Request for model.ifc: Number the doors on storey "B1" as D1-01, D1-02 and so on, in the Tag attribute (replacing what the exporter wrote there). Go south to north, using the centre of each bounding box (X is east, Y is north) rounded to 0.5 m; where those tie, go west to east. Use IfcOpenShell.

First a look at what the model holds.

```python
import ifcopenshell
import ifcopenshell.util.element
import ifcopenshell.util.placement

model = ifcopenshell.open("model.ifc")
print(model.schema)
storey = next(s for s in model.by_type("IfcBuildingStorey") if s.Name == "B1")
doors = [e for e in ifcopenshell.util.element.get_decomposition(storey) if e.is_a("IfcDoor")]
for e in sorted(doors, key=lambda e: e.id()):
    origin = ifcopenshell.util.placement.get_local_placement(e.ObjectPlacement)[:3, 3]
    print(e.id(), e.Tag, e.Name, origin.round(2) + 0.0, sep=" | ")
```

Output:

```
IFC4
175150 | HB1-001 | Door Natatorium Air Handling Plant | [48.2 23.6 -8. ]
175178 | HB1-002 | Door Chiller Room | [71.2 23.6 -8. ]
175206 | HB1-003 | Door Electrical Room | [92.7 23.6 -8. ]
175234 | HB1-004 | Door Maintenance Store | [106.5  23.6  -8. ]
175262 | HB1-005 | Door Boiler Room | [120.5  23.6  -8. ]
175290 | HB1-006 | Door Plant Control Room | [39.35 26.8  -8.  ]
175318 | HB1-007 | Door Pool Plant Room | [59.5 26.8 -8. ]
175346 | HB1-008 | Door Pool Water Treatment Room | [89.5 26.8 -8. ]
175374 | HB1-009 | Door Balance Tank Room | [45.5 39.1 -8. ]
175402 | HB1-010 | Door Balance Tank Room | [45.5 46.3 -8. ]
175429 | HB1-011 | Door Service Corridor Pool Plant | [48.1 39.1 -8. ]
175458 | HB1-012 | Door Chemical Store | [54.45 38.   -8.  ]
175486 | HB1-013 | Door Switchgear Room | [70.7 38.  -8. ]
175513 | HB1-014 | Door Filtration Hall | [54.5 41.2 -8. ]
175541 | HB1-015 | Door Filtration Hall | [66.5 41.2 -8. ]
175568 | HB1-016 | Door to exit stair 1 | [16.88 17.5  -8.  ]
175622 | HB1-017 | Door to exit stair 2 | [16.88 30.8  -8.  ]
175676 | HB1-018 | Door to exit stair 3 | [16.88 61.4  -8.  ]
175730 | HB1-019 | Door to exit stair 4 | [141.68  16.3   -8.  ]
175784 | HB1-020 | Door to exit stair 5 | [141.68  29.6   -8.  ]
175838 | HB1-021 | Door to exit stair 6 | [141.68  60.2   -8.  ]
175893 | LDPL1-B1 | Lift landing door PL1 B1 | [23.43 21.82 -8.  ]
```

```python
import ifcopenshell
import ifcopenshell.geom
import ifcopenshell.util.element
import ifcopenshell.util.shape

model = ifcopenshell.open("model.ifc")
settings = ifcopenshell.geom.settings()
settings.set("use-world-coords", True)


def centre(element):
    shape = ifcopenshell.geom.create_shape(settings, element)
    return ifcopenshell.util.shape.get_bbox_centroid(shape.geometry)


storey = next(s for s in model.by_type("IfcBuildingStorey") if s.Name == "B1")
doors = [e for e in ifcopenshell.util.element.get_decomposition(storey) if e.is_a("IfcDoor")]

# Insertion points can sit at a corner or the storey origin, so sort by the geometry (in metres).
centres = {e: centre(e) for e in doors}
doors.sort(key=lambda e: (round(centres[e][1] / 0.5), centres[e][0]))

for i, e in enumerate(doors, start=1):
    number = f"D1-{i:02d}"
    e.Tag = number
    print(e.id(), number)

model.write("model_v2.ifc")
```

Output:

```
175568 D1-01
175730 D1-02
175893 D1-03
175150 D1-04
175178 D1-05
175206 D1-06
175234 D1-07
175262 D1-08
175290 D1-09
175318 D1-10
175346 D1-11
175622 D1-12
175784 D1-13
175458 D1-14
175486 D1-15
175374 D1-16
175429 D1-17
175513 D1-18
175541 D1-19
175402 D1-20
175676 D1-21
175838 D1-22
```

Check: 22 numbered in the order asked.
